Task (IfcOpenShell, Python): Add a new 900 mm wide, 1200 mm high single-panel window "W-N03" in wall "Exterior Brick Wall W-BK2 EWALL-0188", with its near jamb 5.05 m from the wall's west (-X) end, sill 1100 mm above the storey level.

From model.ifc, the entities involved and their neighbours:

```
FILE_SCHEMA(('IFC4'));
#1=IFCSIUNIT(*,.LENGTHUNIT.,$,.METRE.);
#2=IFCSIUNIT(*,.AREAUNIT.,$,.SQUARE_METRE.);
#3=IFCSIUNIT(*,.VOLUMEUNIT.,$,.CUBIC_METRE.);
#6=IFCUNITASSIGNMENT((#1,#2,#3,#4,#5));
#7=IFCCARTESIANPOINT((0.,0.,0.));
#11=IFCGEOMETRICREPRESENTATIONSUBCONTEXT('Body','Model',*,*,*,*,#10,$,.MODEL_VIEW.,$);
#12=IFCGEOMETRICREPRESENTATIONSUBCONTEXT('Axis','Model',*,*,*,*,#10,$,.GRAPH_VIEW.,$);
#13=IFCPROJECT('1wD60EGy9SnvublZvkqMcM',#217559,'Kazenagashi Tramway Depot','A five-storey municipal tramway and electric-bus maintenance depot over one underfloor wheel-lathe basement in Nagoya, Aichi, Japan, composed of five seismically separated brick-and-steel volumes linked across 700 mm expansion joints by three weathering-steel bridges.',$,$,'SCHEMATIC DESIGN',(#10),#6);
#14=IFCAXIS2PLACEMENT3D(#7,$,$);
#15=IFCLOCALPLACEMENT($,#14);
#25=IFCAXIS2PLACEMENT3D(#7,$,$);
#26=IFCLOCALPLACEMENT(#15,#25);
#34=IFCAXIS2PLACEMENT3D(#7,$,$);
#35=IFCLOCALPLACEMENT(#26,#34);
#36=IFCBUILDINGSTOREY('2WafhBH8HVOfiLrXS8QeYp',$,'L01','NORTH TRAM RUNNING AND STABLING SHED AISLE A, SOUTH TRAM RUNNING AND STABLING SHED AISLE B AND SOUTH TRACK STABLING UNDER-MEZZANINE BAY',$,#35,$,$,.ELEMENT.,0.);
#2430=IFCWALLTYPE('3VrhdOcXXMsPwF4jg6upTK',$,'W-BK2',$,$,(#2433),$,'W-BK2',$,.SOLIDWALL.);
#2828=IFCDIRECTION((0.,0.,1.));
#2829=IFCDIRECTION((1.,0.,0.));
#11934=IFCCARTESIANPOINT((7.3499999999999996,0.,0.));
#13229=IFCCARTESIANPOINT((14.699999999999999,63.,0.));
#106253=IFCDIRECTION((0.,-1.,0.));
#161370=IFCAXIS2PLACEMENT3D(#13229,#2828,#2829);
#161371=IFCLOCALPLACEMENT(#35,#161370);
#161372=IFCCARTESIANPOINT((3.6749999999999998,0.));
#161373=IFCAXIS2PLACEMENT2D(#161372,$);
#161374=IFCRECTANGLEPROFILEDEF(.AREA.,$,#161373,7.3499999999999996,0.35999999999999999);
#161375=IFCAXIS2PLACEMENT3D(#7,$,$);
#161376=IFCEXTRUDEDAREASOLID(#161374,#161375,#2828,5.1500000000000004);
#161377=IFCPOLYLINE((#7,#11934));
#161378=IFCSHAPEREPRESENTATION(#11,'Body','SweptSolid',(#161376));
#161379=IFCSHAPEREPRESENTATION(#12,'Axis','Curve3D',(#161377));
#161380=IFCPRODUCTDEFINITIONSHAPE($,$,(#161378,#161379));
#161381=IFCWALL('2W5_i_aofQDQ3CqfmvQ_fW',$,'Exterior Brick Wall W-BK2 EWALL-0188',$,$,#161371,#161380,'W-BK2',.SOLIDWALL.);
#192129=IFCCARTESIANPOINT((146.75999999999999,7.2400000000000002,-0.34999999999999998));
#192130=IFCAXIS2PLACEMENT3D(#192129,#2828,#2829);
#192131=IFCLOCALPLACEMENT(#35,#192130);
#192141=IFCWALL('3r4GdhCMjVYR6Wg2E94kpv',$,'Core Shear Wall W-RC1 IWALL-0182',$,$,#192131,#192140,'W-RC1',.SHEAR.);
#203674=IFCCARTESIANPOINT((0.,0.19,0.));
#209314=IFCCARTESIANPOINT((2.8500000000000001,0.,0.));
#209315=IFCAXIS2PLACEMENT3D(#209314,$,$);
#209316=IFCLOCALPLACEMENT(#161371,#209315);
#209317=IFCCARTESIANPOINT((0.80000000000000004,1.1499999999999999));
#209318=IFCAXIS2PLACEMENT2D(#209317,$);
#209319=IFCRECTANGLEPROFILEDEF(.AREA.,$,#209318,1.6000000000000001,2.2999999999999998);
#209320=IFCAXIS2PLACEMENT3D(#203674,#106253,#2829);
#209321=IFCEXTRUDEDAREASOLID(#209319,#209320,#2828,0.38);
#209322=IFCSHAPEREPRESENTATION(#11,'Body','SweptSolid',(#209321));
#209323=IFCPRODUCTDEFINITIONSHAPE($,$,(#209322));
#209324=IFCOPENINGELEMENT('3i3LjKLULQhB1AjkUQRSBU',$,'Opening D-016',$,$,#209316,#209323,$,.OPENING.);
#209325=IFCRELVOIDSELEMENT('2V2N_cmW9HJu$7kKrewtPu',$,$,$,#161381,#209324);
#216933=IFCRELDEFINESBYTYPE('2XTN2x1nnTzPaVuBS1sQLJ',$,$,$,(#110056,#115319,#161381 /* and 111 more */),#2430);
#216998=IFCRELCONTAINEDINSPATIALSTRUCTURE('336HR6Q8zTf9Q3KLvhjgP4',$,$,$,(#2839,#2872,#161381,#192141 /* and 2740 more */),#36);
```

```python
import numpy as np
import ifcopenshell
import ifcopenshell.api.feature
import ifcopenshell.api.geometry
import ifcopenshell.api.root
import ifcopenshell.api.spatial
import ifcopenshell.geom
import ifcopenshell.util.element
import ifcopenshell.util.placement
import ifcopenshell.util.representation
import ifcopenshell.util.shape
import ifcopenshell.util.unit

model = ifcopenshell.open("model.ifc")
unit_scale = ifcopenshell.util.unit.calculate_unit_scale(model)
settings = ifcopenshell.geom.settings()


def volume(element):
    """Net volume in cubic metres, openings subtracted."""
    shape = ifcopenshell.geom.create_shape(settings, element)
    return ifcopenshell.util.shape.get_volume(shape.geometry)


wall = model.by_guid("2W5_i_aofQDQ3CqfmvQ_fW")
storey = ifcopenshell.util.element.get_container(wall, ifc_class="IfcBuildingStorey")
context = ifcopenshell.util.representation.get_context(model, "Model", "Body", "MODEL_VIEW")
before = volume(wall)

width, height, from_end, sill = 0.9, 1.2, 5.05, 1.1  # metres

# The wall runs along its own X axis, and the end named is its -X end.
wall_shape = ifcopenshell.geom.create_shape(settings, wall)
x, y, z = ifcopenshell.util.shape.get_vertices(wall_shape.geometry).T
start = x.min() + from_end
face, thickness = float(y.min()), float(y.max() - y.min())
wall_matrix = ifcopenshell.util.placement.get_local_placement(wall.ObjectPlacement)
level = ifcopenshell.util.placement.get_local_placement(storey.ObjectPlacement)[2, 3]


def in_wall(x, y):
    """Placement at x, y metres in the wall's axes, at sill height."""
    matrix = wall_matrix.copy()
    matrix[:, 3] = wall_matrix @ np.array([x / unit_scale, y / unit_scale, 0.0, 1.0])
    matrix[2, 3] = level + sill / unit_scale
    return matrix


# Opening: a box that overshoots both wall faces by 50 mm.
opening = ifcopenshell.api.root.create_entity(model, ifc_class="IfcOpeningElement", predefined_type="OPENING")
box = ifcopenshell.api.geometry.add_wall_representation(
    model, context=context, length=width, height=height, thickness=thickness + 0.1
)
ifcopenshell.api.geometry.assign_representation(model, product=opening, representation=box)
ifcopenshell.api.geometry.edit_object_placement(model, product=opening, matrix=in_wall(start, face - 0.05), is_si=False)
ifcopenshell.api.feature.add_feature(model, feature=opening, element=wall)

window = ifcopenshell.api.root.create_entity(model, ifc_class="IfcWindow", name="W-N03", predefined_type="WINDOW")
window.OverallWidth, window.OverallHeight = width / unit_scale, height / unit_scale
window.PartitioningType = "SINGLE_PANEL"
body = ifcopenshell.api.geometry.add_window_representation(
    model,
    context=context,
    overall_width=window.OverallWidth,
    overall_height=window.OverallHeight,
    partition_type="SINGLE_PANEL",
)
ifcopenshell.api.geometry.assign_representation(model, product=window, representation=body)
ifcopenshell.api.spatial.assign_container(model, products=[window], relating_structure=storey)
ifcopenshell.api.feature.add_filling(model, opening=opening, element=window)

# Centre the window in the wall's thickness.
ifcopenshell.api.geometry.edit_object_placement(model, product=window, matrix=in_wall(start, face), is_si=False)
window_shape = ifcopenshell.geom.create_shape(settings, window)
depth = ifcopenshell.util.shape.get_vertices(window_shape.geometry)[:, 1]
offset = face + thickness / 2 - (depth.min() + depth.max()) / 2
ifcopenshell.api.geometry.edit_object_placement(model, product=window, matrix=in_wall(start, offset), is_si=False)

after = volume(wall)

print(f"wall volume {before:.3f} -> {after:.3f} m3")

model.write("model_edited.ifc")
```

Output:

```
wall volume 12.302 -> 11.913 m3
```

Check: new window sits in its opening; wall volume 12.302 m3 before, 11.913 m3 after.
